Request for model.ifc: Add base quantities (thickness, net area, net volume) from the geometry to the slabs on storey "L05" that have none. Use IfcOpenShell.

First a look at what the model holds.

```python
import ifcopenshell
import ifcopenshell.util.element
import ifcopenshell.util.unit

model = ifcopenshell.open("model.ifc")
print(model.schema)
for unit_type in ("LENGTHUNIT", "AREAUNIT", "VOLUMEUNIT"):
    print(unit_type, ifcopenshell.util.unit.calculate_unit_scale(model, unit_type))
storey = next(s for s in model.by_type("IfcBuildingStorey") if s.Name == "L05")
slabs = [e for e in ifcopenshell.util.element.get_decomposition(storey) if e.is_a("IfcSlab")]
for e in sorted(slabs, key=lambda e: e.id()):
    print(e.id(), e.is_a(), e.Name, list(ifcopenshell.util.element.get_psets(e, qtos_only=True)), sep=" | ")
```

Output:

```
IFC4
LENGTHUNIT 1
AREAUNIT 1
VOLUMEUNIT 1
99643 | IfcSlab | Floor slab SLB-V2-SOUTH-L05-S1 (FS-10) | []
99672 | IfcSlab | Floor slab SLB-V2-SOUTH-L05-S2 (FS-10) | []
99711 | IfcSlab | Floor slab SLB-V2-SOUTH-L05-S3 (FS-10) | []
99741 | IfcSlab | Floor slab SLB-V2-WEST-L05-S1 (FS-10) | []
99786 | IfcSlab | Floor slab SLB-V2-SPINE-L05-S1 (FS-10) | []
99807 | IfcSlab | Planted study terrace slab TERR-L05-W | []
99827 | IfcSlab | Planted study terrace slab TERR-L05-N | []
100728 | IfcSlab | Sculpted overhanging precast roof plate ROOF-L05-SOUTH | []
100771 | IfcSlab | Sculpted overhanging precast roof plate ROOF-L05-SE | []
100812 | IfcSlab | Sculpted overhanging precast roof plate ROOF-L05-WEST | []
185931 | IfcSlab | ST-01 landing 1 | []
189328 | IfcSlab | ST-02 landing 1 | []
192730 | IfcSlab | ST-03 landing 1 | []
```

```python
import ifcopenshell
import ifcopenshell.api.pset
import ifcopenshell.geom
import ifcopenshell.util.element
import ifcopenshell.util.shape
import ifcopenshell.util.unit

model = ifcopenshell.open("model.ifc")
unit_scale = ifcopenshell.util.unit.calculate_unit_scale(model)
area_scale = ifcopenshell.util.unit.calculate_unit_scale(model, "AREAUNIT")
volume_scale = ifcopenshell.util.unit.calculate_unit_scale(model, "VOLUMEUNIT")
settings = ifcopenshell.geom.settings()

storey = next(s for s in model.by_type("IfcBuildingStorey") if s.Name == "L05")
slabs = [e for e in ifcopenshell.util.element.get_decomposition(storey) if e.is_a("IfcSlab")]

for e in sorted(slabs, key=lambda e: e.id()):
    if ifcopenshell.util.element.get_psets(e, qtos_only=True, should_inherit=False):
        continue
    # Geometry comes back in metres, in the element's own axes.
    shape = ifcopenshell.geom.create_shape(settings, e)
    values = {
        "Width": ifcopenshell.util.shape.get_z(shape.geometry) / unit_scale,
        "NetArea": ifcopenshell.util.shape.get_footprint_area(shape.geometry) / area_scale,
        "NetVolume": ifcopenshell.util.shape.get_volume(shape.geometry) / volume_scale,
    }
    qto = ifcopenshell.api.pset.add_qto(model, product=e, name="Qto_SlabBaseQuantities")
    ifcopenshell.api.pset.edit_qto(model, qto=qto, properties=values)
    print(e.id(), {k: round(v, 3) for k, v in values.items()})

model.write("model_rev.ifc")
```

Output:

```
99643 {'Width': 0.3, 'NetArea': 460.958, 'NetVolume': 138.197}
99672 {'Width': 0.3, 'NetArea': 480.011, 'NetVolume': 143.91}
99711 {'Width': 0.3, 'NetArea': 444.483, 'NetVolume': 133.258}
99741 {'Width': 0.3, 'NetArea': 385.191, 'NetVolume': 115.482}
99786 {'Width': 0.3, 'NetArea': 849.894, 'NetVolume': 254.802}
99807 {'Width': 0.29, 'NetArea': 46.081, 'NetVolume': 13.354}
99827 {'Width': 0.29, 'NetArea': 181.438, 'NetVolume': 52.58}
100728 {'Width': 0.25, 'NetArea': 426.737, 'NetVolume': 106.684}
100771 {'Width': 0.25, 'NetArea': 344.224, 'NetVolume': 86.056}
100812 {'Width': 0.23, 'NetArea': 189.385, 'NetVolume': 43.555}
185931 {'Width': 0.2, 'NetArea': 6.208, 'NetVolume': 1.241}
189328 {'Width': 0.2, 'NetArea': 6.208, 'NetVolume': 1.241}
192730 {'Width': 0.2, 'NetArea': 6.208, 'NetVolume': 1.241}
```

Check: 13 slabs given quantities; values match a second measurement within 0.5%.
